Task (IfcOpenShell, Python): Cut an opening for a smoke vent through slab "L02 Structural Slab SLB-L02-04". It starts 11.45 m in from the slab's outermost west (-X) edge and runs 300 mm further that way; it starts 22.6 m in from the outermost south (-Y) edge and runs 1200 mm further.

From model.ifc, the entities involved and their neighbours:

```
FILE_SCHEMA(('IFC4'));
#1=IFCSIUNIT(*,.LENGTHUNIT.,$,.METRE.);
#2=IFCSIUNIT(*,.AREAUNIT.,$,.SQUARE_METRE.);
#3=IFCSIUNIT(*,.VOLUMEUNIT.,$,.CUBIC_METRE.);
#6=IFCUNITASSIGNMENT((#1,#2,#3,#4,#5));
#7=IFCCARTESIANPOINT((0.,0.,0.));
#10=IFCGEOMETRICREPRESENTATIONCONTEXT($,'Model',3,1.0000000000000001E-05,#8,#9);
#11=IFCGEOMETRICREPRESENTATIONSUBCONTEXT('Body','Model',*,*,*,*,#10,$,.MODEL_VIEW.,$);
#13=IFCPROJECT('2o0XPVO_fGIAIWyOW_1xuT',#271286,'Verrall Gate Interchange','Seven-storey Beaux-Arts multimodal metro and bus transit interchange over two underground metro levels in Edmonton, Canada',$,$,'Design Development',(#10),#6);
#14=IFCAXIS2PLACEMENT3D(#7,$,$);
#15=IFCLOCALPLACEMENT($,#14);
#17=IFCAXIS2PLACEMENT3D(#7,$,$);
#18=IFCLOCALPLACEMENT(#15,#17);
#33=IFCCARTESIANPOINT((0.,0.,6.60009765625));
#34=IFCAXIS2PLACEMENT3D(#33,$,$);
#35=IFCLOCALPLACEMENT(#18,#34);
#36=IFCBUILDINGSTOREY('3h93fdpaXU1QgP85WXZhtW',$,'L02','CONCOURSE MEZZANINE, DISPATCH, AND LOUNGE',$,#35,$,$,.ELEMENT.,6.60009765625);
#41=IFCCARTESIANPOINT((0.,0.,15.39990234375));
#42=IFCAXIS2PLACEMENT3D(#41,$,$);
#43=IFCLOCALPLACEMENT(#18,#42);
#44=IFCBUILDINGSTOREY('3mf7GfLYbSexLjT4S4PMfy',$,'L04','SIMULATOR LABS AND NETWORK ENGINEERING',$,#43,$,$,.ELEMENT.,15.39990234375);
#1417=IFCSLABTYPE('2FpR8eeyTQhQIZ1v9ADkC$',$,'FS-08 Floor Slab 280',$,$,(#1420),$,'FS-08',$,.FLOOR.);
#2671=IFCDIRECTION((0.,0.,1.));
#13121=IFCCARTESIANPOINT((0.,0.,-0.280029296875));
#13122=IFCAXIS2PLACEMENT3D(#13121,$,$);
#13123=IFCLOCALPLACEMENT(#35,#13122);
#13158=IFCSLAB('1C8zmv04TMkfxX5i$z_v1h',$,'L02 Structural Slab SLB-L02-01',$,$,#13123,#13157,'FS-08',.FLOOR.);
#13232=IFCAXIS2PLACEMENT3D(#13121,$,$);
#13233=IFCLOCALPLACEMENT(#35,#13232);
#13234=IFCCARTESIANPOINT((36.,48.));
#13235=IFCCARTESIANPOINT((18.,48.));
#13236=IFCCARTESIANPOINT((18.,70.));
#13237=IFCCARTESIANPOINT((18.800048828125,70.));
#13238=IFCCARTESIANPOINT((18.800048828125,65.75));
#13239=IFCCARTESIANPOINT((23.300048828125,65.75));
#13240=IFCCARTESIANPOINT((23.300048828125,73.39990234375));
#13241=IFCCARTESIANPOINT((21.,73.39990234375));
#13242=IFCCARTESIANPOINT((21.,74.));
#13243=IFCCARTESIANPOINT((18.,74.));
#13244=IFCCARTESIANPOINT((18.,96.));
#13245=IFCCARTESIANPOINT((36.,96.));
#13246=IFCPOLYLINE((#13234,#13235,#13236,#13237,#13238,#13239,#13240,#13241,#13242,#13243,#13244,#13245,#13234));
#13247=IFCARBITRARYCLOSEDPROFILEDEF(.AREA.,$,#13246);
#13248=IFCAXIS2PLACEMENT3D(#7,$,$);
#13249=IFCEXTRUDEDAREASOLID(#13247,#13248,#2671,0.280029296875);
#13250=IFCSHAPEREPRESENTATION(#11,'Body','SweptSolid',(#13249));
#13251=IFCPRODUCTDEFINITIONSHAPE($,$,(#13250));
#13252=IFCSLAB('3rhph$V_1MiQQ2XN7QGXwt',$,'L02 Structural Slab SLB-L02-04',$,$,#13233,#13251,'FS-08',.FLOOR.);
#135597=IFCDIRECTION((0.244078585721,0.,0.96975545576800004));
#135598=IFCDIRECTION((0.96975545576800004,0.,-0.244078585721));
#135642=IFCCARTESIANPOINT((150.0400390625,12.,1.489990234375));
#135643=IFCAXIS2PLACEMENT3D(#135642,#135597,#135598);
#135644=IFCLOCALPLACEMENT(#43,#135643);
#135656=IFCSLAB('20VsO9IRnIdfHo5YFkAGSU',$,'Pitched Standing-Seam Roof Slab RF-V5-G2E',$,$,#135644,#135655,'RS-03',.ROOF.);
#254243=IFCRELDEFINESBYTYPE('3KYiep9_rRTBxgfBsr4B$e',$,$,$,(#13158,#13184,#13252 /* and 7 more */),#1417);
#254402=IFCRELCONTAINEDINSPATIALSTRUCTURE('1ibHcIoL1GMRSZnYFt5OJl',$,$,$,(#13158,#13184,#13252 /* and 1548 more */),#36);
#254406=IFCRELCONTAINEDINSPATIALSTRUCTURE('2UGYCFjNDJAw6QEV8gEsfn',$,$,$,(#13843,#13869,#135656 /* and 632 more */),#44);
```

```python
import numpy as np
import ifcopenshell
import ifcopenshell.api.feature
import ifcopenshell.api.geometry
import ifcopenshell.api.root
import ifcopenshell.geom
import ifcopenshell.util.placement
import ifcopenshell.util.representation
import ifcopenshell.util.shape
import ifcopenshell.util.unit

model = ifcopenshell.open("model.ifc")
unit_scale = ifcopenshell.util.unit.calculate_unit_scale(model)
settings = ifcopenshell.geom.settings()


def volume(element):
    """Net volume in cubic metres, openings subtracted."""
    shape = ifcopenshell.geom.create_shape(settings, element)
    return ifcopenshell.util.shape.get_volume(shape.geometry)


slab = model.by_id(13252)
before = volume(slab)

# Extent in the slab's own axes, in metres. The edges named are its -X and -Y sides.
slab_shape = ifcopenshell.geom.create_shape(settings, slab)
vertices = ifcopenshell.util.shape.get_vertices(slab_shape.geometry)
x_min, y_min, bottom = vertices.min(axis=0)
top = vertices[:, 2].max()

opening = ifcopenshell.api.root.create_entity(model, ifc_class="IfcOpeningElement", name="Smoke vent opening", predefined_type="OPENING")
context = ifcopenshell.util.representation.get_context(model, "Model", "Body", "MODEL_VIEW")
width, depth = 0.3, 1.2
outline = [(0.0, 0.0), (width, 0.0), (width, depth), (0.0, depth), (0.0, 0.0)]
# Overshoot both faces by 50 mm so the cut is clean.
shape = ifcopenshell.api.geometry.add_slab_representation(
    model, context=context, depth=top - bottom + 0.1, polyline=outline
)
ifcopenshell.api.geometry.assign_representation(model, product=opening, representation=shape)

matrix = ifcopenshell.util.placement.get_local_placement(slab.ObjectPlacement)
matrix[:, 3] = matrix @ np.append(np.array([x_min + 11.45, y_min + 22.6, bottom - 0.05]) / unit_scale, 1.0)
ifcopenshell.api.geometry.edit_object_placement(model, product=opening, matrix=matrix, is_si=False)
ifcopenshell.api.feature.add_feature(model, feature=opening, element=slab)

after = volume(slab)

print(f"slab volume {before:.3f} -> {after:.3f} m3")

model.write("model-out.ifc")
```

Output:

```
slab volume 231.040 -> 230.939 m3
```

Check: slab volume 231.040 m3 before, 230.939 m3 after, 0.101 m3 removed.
